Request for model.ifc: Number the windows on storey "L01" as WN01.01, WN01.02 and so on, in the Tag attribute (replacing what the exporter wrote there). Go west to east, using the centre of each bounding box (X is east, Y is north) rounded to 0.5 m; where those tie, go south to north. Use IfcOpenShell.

First a look at what the model holds.

```python
import ifcopenshell
import ifcopenshell.util.element
import ifcopenshell.util.placement

model = ifcopenshell.open("model.ifc")
print(model.schema)
storey = next(s for s in model.by_type("IfcBuildingStorey") if s.Name == "L01")
windows = [e for e in ifcopenshell.util.element.get_decomposition(storey) if e.is_a("IfcWindow")]
for e in sorted(windows, key=lambda e: e.id()):
    origin = ifcopenshell.util.placement.get_local_placement(e.ObjectPlacement)[:3, 3]
    print(e.id(), e.Tag, e.Name, origin.round(2) + 0.0, sep=" | ")
```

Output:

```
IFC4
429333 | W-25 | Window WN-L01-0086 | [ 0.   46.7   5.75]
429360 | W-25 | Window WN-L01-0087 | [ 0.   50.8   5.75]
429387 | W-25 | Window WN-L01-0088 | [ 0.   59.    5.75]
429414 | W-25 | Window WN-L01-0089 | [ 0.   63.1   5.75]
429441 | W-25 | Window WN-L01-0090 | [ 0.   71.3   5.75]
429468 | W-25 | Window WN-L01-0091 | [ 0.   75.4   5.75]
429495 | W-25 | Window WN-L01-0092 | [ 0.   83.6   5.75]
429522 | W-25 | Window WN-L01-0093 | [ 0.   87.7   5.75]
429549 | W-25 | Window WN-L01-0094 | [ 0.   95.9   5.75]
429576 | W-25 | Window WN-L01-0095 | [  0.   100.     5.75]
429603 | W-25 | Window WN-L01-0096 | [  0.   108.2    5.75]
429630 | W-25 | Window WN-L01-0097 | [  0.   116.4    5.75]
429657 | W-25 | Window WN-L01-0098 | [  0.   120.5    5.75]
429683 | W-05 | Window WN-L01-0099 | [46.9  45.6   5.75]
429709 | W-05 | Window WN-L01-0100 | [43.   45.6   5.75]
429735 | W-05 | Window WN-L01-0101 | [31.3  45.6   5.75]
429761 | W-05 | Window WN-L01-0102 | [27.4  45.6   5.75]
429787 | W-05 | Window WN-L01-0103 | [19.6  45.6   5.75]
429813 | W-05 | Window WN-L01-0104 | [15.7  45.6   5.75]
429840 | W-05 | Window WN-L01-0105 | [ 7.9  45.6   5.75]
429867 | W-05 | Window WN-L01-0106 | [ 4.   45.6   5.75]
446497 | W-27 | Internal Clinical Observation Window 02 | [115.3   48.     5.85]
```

```python
import ifcopenshell
import ifcopenshell.geom
import ifcopenshell.util.element
import ifcopenshell.util.shape

model = ifcopenshell.open("model.ifc")
settings = ifcopenshell.geom.settings()
settings.set("use-world-coords", True)


def centre(element):
    shape = ifcopenshell.geom.create_shape(settings, element)
    return ifcopenshell.util.shape.get_bbox_centroid(shape.geometry)


storey = next(s for s in model.by_type("IfcBuildingStorey") if s.Name == "L01")
windows = [e for e in ifcopenshell.util.element.get_decomposition(storey) if e.is_a("IfcWindow")]

# Insertion points can sit at a corner or the storey origin, so sort by the geometry (in metres).
centres = {e: centre(e) for e in windows}
windows.sort(key=lambda e: (round(centres[e][0] / 0.5), centres[e][1]))

for i, e in enumerate(windows, start=1):
    number = f"WN01.{i:02d}"
    e.Tag = number
    print(e.id(), number)

model.write("model_edited.ifc")
```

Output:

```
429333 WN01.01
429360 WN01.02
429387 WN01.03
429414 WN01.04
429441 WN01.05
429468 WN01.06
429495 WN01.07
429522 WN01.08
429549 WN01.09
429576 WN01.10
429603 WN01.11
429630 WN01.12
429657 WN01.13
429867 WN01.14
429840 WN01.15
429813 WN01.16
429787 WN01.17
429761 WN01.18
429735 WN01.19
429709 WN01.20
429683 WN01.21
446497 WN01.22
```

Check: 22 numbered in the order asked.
